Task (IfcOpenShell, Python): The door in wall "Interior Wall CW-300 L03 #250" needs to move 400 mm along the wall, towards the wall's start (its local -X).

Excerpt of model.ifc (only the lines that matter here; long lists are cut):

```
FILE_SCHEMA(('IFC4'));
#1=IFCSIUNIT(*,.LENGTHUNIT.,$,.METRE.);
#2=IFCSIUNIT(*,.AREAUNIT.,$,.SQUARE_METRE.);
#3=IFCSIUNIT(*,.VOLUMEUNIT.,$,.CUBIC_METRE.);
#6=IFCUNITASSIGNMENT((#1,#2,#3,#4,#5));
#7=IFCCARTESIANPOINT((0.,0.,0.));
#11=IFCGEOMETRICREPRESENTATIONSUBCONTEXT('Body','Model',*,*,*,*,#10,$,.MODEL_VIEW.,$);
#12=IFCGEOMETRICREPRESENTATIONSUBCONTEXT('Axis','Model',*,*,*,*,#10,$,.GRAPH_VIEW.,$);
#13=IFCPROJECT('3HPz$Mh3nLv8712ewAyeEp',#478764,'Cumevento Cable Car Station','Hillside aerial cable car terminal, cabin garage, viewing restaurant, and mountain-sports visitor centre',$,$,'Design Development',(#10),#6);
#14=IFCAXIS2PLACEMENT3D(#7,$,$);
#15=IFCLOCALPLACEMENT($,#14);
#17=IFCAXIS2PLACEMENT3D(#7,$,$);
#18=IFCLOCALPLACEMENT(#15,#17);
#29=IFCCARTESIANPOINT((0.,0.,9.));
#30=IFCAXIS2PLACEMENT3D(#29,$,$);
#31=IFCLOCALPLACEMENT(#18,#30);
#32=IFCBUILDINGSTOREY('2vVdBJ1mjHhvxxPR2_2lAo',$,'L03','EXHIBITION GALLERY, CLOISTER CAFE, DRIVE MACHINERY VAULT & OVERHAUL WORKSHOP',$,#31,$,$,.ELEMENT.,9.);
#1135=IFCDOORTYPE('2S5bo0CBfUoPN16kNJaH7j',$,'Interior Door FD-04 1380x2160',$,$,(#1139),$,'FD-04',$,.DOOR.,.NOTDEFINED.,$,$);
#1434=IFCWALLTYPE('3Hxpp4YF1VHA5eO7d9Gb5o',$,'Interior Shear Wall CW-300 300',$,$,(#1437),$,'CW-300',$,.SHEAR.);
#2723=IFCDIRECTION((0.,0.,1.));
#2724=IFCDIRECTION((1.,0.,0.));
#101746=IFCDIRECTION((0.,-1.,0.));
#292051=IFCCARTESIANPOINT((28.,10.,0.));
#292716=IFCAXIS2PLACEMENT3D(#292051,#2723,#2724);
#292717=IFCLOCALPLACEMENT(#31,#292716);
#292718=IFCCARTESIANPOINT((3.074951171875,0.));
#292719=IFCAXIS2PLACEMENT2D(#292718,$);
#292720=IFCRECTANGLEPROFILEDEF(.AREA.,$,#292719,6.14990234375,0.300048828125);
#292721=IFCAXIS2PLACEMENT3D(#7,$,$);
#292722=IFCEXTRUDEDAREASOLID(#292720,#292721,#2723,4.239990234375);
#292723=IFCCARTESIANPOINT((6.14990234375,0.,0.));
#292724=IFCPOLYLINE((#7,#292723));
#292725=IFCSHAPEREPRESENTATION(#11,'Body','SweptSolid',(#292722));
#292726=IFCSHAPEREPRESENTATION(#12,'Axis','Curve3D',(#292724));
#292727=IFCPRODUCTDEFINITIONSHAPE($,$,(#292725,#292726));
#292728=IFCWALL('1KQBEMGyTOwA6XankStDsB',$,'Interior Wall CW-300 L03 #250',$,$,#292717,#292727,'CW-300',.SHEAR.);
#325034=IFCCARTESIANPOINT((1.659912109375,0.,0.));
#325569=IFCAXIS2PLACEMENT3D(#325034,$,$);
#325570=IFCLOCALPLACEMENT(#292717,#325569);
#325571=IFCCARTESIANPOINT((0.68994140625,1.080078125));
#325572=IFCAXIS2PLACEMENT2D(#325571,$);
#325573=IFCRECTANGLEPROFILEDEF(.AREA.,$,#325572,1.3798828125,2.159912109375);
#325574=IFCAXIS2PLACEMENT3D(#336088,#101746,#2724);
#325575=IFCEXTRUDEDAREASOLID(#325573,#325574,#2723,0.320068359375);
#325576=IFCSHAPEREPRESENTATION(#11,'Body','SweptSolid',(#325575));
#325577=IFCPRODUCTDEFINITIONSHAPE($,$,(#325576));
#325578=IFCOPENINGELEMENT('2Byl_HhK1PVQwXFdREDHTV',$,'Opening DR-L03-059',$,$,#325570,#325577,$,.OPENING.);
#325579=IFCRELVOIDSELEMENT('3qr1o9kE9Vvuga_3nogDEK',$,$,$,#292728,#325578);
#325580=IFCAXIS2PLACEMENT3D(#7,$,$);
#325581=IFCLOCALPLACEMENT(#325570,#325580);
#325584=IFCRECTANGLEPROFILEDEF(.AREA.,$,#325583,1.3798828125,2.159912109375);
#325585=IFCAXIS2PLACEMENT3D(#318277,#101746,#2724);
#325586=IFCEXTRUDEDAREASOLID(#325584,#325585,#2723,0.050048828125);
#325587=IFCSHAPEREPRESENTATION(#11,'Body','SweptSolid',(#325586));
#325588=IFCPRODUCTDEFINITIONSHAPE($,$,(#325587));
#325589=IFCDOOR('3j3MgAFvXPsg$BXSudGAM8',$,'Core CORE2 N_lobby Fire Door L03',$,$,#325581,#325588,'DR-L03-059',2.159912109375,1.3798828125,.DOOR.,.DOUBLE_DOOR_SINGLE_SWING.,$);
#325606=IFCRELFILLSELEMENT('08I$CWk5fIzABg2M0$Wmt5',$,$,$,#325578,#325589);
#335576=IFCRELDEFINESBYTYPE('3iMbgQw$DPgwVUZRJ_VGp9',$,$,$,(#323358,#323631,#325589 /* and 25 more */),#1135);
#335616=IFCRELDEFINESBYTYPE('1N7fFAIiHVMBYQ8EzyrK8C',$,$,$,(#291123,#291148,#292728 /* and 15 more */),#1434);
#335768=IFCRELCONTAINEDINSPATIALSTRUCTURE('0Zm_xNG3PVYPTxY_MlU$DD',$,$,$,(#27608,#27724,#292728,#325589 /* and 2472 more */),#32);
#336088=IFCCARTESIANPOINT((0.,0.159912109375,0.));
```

```python
import ifcopenshell
import ifcopenshell.api.geometry
import ifcopenshell.util.placement

model = ifcopenshell.open("model.ifc")

door = model.by_id(325589)
opening = door.FillsVoids[0].RelatingOpeningElement
wall = opening.VoidsElements[0].RelatingBuildingElement

wall_matrix = ifcopenshell.util.placement.get_local_placement(wall.ObjectPlacement)
shift = wall_matrix[:3, 0] * -0.4
before = ifcopenshell.util.placement.get_local_placement(door.ObjectPlacement)[:3, 3].copy()

# The door is placed relative to its opening, so it follows when the opening moves.
matrix = ifcopenshell.util.placement.get_local_placement(opening.ObjectPlacement)
matrix[:3, 3] += shift
ifcopenshell.api.geometry.edit_object_placement(
    model, product=opening, matrix=matrix, is_si=False, should_transform_children=True
)

after = ifcopenshell.util.placement.get_local_placement(door.ObjectPlacement)[:3, 3]
print("door moved by", (after - before).round(3) + 0.0)

model.write("model_rev.ifc")
```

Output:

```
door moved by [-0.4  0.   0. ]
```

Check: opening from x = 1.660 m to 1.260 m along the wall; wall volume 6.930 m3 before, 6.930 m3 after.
